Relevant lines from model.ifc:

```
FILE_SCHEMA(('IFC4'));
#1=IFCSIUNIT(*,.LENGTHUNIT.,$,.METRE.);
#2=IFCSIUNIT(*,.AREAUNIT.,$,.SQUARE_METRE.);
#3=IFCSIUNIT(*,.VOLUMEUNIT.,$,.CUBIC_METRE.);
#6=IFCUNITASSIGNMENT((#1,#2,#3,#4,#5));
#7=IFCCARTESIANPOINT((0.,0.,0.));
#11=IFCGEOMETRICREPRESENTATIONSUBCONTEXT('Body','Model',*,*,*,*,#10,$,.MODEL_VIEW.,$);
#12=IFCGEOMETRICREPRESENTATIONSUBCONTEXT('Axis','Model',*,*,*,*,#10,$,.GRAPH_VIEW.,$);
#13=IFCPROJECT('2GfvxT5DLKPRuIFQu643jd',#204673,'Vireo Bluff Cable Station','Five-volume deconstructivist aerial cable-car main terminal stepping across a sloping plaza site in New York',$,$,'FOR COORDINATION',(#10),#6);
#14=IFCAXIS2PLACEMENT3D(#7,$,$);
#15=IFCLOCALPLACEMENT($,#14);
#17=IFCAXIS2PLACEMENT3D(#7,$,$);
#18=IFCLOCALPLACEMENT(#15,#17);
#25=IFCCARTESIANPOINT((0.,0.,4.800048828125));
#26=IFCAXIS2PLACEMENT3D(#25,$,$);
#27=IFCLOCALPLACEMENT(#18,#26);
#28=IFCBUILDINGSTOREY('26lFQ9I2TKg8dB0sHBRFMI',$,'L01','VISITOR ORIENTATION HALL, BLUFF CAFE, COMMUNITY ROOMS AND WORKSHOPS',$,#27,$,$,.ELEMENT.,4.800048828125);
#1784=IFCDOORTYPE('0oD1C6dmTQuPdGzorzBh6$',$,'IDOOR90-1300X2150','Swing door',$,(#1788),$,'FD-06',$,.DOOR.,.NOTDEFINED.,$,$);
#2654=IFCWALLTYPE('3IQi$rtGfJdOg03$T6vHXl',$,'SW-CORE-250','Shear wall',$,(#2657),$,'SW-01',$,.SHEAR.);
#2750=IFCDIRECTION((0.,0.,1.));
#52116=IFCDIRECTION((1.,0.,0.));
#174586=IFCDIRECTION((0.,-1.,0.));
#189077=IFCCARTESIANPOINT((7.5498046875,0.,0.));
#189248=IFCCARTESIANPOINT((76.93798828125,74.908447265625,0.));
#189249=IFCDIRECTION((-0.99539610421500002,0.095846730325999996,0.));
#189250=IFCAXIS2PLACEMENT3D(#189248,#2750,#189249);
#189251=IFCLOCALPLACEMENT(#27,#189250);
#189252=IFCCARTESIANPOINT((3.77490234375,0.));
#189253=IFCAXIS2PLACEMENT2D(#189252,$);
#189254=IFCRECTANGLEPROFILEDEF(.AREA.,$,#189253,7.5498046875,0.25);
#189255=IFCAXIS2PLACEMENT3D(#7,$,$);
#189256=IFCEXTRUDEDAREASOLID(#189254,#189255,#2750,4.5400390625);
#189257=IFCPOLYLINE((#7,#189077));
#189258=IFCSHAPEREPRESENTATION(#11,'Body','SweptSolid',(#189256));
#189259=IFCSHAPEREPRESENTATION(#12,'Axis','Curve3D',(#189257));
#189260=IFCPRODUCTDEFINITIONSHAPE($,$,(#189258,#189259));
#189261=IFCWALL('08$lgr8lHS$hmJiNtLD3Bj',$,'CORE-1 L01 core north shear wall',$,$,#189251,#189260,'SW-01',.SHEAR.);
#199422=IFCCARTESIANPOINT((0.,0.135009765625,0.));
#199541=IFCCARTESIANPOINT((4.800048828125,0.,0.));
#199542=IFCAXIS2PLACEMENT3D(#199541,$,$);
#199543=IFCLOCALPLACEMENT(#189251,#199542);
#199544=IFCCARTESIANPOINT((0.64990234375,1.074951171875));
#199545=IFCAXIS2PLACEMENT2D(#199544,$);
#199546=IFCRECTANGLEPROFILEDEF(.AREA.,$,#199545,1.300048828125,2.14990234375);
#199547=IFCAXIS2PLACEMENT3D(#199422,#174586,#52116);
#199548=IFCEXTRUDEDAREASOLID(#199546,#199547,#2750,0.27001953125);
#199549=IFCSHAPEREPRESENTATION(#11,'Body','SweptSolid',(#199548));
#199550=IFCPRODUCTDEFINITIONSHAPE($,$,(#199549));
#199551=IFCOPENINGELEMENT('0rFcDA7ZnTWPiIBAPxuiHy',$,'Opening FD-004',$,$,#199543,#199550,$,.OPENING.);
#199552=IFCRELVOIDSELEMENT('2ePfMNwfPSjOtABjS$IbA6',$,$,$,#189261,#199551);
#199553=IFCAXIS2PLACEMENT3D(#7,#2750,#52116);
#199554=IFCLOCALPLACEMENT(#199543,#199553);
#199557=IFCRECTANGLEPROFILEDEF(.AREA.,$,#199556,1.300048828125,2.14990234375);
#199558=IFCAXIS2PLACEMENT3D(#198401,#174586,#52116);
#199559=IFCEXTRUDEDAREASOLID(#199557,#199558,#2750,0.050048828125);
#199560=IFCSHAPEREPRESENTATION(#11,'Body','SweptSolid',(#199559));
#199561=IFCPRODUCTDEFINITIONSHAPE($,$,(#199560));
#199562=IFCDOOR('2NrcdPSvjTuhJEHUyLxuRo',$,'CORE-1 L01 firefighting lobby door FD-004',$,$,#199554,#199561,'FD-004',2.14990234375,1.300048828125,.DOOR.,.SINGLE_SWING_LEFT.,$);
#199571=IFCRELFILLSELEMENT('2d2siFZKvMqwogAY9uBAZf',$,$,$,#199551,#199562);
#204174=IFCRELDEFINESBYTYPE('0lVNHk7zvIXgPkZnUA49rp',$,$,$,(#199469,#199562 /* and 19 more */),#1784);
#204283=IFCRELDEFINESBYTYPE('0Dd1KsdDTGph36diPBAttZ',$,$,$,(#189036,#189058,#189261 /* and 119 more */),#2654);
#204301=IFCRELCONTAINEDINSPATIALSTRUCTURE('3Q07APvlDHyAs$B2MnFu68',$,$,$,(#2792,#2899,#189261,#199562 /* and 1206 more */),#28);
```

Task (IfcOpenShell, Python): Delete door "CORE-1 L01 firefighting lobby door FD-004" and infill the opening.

```python
import ifcopenshell
import ifcopenshell.api.feature
import ifcopenshell.api.root
import ifcopenshell.geom
import ifcopenshell.util.shape

model = ifcopenshell.open("model.ifc")
settings = ifcopenshell.geom.settings()


def volume(element):
    """Net volume in cubic metres, openings subtracted."""
    shape = ifcopenshell.geom.create_shape(settings, element)
    return ifcopenshell.util.shape.get_volume(shape.geometry)


door = model.by_guid("2NrcdPSvjTuhJEHUyLxuRo")
opening = door.FillsVoids[0].RelatingOpeningElement
wall = opening.VoidsElements[0].RelatingBuildingElement
before = volume(wall)

ifcopenshell.api.root.remove_product(model, product=door)
ifcopenshell.api.feature.remove_feature(model, feature=opening)

after = volume(wall)

print(f"wall volume {before:.3f} -> {after:.3f} m3")

model.write("model_updated.ifc")
```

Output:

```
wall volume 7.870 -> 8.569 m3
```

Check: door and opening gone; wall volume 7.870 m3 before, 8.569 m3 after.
